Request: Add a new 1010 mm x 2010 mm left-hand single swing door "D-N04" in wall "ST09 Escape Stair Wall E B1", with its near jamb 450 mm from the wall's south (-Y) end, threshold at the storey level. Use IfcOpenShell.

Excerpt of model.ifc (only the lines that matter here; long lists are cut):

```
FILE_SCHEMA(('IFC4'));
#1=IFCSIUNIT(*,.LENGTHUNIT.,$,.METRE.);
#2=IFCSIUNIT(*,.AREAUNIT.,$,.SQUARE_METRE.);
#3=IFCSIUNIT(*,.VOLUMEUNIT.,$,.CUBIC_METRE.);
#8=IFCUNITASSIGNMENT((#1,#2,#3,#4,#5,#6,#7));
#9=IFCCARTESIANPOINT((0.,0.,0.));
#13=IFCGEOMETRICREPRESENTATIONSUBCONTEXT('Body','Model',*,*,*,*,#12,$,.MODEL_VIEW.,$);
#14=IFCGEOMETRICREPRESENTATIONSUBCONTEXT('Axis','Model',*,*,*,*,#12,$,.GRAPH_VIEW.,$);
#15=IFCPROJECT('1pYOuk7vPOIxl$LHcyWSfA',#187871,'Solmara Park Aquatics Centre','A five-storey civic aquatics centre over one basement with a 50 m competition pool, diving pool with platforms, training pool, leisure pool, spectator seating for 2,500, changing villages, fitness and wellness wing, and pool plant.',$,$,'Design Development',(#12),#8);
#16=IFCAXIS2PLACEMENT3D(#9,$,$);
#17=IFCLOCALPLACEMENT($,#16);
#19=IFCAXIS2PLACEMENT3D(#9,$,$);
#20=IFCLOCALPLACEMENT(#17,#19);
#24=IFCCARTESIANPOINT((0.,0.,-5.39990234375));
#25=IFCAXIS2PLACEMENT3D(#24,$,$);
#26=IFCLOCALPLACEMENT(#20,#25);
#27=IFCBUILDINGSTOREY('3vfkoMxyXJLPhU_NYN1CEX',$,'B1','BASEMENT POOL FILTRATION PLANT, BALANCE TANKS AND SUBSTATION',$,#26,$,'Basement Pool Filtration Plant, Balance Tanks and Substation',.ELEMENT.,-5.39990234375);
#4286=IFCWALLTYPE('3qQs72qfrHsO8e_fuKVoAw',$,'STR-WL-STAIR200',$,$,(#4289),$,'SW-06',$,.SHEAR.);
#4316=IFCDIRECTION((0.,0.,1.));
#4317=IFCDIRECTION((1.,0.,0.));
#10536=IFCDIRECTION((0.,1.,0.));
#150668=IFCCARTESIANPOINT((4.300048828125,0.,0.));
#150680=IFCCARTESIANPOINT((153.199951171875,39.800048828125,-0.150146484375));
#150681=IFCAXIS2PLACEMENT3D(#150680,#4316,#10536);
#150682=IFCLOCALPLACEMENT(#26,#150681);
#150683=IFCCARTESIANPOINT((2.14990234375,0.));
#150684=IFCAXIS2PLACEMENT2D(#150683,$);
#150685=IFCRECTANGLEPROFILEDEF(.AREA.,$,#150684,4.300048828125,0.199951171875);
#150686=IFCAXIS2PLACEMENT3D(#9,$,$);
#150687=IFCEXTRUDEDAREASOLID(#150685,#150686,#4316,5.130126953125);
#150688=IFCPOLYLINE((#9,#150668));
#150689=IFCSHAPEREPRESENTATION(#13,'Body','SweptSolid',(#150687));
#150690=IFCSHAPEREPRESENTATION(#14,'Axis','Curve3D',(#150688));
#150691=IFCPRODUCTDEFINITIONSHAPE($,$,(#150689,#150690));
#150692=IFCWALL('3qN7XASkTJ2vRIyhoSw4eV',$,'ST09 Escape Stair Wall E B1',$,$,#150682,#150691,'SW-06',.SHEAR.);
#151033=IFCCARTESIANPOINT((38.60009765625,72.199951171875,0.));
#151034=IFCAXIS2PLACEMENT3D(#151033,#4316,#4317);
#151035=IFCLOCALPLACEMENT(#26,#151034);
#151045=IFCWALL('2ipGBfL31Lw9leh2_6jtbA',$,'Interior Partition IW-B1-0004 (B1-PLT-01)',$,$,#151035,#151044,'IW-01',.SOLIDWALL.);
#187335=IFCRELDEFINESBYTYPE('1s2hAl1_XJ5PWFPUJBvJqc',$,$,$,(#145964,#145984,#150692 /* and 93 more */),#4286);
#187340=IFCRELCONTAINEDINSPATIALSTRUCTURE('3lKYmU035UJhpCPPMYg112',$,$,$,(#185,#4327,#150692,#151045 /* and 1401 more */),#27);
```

```python
import numpy as np
import ifcopenshell
import ifcopenshell.api.feature
import ifcopenshell.api.geometry
import ifcopenshell.api.root
import ifcopenshell.api.spatial
import ifcopenshell.geom
import ifcopenshell.util.element
import ifcopenshell.util.placement
import ifcopenshell.util.representation
import ifcopenshell.util.shape
import ifcopenshell.util.unit

model = ifcopenshell.open("model.ifc")
unit_scale = ifcopenshell.util.unit.calculate_unit_scale(model)
settings = ifcopenshell.geom.settings()


def volume(element):
    """Net volume in cubic metres, openings subtracted."""
    shape = ifcopenshell.geom.create_shape(settings, element)
    return ifcopenshell.util.shape.get_volume(shape.geometry)


wall = model.by_guid("3qN7XASkTJ2vRIyhoSw4eV")
storey = ifcopenshell.util.element.get_container(wall, ifc_class="IfcBuildingStorey")
context = ifcopenshell.util.representation.get_context(model, "Model", "Body", "MODEL_VIEW")
before = volume(wall)

width, height, from_end, sill = 1.01, 2.01, 0.45, 0.0  # metres

# The wall runs along its own X axis, and the end named is its -X end.
wall_shape = ifcopenshell.geom.create_shape(settings, wall)
x, y, z = ifcopenshell.util.shape.get_vertices(wall_shape.geometry).T
start = x.min() + from_end
face, thickness = float(y.min()), float(y.max() - y.min())
wall_matrix = ifcopenshell.util.placement.get_local_placement(wall.ObjectPlacement)
level = ifcopenshell.util.placement.get_local_placement(storey.ObjectPlacement)[2, 3]


def in_wall(x, y):
    """Placement at x, y metres in the wall's axes, at sill height."""
    matrix = wall_matrix.copy()
    matrix[:, 3] = wall_matrix @ np.array([x / unit_scale, y / unit_scale, 0.0, 1.0])
    matrix[2, 3] = level + sill / unit_scale
    return matrix


# Opening: a box that overshoots both wall faces by 50 mm.
opening = ifcopenshell.api.root.create_entity(model, ifc_class="IfcOpeningElement", predefined_type="OPENING")
box = ifcopenshell.api.geometry.add_wall_representation(
    model, context=context, length=width, height=height, thickness=thickness + 0.1
)
ifcopenshell.api.geometry.assign_representation(model, product=opening, representation=box)
ifcopenshell.api.geometry.edit_object_placement(model, product=opening, matrix=in_wall(start, face - 0.05), is_si=False)
ifcopenshell.api.feature.add_feature(model, feature=opening, element=wall)

door = ifcopenshell.api.root.create_entity(model, ifc_class="IfcDoor", name="D-N04", predefined_type="DOOR")
door.OverallWidth, door.OverallHeight = width / unit_scale, height / unit_scale
door.OperationType = "SINGLE_SWING_LEFT"
body = ifcopenshell.api.geometry.add_door_representation(
    model,
    context=context,
    overall_width=door.OverallWidth,
    overall_height=door.OverallHeight,
    operation_type="SINGLE_SWING_LEFT",
    lining_properties={"LiningDepth": thickness / unit_scale, "ThresholdDepth": thickness / unit_scale},
)
ifcopenshell.api.geometry.assign_representation(model, product=door, representation=body)
ifcopenshell.api.spatial.assign_container(model, products=[door], relating_structure=storey)
ifcopenshell.api.feature.add_filling(model, opening=opening, element=door)

# The lining spans the wall, so the door starts at the wall face.
ifcopenshell.api.geometry.edit_object_placement(model, product=door, matrix=in_wall(start, face), is_si=False)

after = volume(wall)

print(f"wall volume {before:.3f} -> {after:.3f} m3")

model.write("model_rev.ifc")
```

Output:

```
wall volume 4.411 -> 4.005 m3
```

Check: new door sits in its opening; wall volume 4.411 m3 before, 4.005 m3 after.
